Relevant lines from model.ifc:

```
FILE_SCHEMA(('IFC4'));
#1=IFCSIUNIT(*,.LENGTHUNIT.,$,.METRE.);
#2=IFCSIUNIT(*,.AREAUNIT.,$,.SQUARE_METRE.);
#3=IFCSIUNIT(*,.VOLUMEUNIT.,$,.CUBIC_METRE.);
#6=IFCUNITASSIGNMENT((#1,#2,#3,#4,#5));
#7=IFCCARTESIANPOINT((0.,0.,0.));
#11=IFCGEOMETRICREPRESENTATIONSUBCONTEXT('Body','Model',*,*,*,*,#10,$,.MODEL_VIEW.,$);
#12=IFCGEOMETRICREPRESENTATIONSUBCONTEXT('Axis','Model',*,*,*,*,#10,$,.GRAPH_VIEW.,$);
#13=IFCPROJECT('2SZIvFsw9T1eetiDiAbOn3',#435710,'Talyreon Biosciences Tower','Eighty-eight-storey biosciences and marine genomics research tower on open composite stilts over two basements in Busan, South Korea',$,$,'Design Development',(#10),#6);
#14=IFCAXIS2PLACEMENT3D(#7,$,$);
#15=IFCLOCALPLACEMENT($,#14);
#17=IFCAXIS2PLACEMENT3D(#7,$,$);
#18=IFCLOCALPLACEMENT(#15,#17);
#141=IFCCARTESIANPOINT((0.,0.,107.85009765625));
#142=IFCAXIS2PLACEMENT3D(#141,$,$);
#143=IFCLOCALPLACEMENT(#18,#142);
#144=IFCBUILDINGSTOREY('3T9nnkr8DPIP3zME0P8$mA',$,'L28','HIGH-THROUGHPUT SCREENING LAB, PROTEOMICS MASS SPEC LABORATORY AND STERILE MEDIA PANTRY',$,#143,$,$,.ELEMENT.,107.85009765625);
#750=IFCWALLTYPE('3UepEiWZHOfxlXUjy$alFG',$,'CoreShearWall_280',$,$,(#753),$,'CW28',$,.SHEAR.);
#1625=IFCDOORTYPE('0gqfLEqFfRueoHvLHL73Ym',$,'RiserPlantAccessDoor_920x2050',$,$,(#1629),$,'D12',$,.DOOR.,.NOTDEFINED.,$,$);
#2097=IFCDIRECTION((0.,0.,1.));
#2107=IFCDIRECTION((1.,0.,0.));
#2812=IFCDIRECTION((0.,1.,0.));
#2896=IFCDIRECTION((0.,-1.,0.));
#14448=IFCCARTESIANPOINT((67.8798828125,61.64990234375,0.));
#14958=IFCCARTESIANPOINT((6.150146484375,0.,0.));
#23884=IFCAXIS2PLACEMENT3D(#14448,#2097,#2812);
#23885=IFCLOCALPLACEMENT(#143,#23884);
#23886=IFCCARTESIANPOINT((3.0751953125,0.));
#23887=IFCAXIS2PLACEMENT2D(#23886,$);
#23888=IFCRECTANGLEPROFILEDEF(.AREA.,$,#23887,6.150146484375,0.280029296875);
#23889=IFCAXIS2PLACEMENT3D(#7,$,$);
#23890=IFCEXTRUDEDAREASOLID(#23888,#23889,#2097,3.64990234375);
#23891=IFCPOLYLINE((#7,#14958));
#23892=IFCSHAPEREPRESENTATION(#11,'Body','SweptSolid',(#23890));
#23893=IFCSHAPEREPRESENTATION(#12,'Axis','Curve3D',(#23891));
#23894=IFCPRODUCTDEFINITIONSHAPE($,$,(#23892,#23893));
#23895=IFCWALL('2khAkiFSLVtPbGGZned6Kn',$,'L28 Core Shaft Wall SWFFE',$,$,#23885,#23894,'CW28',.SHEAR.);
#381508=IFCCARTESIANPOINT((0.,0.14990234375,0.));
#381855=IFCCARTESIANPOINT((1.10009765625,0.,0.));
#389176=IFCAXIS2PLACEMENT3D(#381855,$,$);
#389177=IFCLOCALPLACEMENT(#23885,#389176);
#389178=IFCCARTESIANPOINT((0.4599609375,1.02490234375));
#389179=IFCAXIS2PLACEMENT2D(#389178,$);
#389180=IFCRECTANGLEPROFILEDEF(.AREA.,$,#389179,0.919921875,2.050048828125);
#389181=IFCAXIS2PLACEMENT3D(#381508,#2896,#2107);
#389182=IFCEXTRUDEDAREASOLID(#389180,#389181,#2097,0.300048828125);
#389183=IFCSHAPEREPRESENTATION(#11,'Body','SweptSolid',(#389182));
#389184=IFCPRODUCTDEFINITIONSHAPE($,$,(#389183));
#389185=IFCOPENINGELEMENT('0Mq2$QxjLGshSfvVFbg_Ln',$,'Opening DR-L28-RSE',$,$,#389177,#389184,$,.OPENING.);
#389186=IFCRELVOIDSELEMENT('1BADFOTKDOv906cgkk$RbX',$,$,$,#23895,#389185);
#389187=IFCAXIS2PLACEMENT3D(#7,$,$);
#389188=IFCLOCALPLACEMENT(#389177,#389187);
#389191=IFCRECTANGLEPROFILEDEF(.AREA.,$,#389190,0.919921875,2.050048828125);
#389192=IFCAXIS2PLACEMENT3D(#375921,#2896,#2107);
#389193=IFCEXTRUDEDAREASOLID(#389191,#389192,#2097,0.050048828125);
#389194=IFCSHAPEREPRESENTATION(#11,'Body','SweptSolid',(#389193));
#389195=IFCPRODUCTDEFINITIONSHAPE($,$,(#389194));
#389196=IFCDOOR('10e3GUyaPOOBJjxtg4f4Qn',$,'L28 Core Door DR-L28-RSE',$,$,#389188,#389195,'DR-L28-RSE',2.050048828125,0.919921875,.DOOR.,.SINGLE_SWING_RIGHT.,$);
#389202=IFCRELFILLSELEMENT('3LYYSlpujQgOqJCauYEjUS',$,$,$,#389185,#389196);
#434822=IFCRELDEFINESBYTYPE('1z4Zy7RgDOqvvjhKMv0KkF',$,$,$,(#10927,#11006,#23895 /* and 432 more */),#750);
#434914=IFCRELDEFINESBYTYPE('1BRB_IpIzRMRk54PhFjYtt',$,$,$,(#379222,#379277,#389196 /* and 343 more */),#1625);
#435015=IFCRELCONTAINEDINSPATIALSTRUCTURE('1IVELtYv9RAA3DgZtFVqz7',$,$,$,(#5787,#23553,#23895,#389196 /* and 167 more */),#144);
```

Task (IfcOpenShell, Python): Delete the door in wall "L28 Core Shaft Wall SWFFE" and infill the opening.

```python
import ifcopenshell
import ifcopenshell.api.feature
import ifcopenshell.api.root
import ifcopenshell.geom
import ifcopenshell.util.shape

model = ifcopenshell.open("model.ifc")
settings = ifcopenshell.geom.settings()


def volume(element):
    """Net volume in cubic metres, openings subtracted."""
    shape = ifcopenshell.geom.create_shape(settings, element)
    return ifcopenshell.util.shape.get_volume(shape.geometry)


door = model.by_guid("10e3GUyaPOOBJjxtg4f4Qn")
opening = door.FillsVoids[0].RelatingOpeningElement
wall = opening.VoidsElements[0].RelatingBuildingElement
before = volume(wall)

ifcopenshell.api.root.remove_product(model, product=door)
ifcopenshell.api.feature.remove_feature(model, feature=opening)

after = volume(wall)

print(f"wall volume {before:.3f} -> {after:.3f} m3")

model.write("model_rev.ifc")
```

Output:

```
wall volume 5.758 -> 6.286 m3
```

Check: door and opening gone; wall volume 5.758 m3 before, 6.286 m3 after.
